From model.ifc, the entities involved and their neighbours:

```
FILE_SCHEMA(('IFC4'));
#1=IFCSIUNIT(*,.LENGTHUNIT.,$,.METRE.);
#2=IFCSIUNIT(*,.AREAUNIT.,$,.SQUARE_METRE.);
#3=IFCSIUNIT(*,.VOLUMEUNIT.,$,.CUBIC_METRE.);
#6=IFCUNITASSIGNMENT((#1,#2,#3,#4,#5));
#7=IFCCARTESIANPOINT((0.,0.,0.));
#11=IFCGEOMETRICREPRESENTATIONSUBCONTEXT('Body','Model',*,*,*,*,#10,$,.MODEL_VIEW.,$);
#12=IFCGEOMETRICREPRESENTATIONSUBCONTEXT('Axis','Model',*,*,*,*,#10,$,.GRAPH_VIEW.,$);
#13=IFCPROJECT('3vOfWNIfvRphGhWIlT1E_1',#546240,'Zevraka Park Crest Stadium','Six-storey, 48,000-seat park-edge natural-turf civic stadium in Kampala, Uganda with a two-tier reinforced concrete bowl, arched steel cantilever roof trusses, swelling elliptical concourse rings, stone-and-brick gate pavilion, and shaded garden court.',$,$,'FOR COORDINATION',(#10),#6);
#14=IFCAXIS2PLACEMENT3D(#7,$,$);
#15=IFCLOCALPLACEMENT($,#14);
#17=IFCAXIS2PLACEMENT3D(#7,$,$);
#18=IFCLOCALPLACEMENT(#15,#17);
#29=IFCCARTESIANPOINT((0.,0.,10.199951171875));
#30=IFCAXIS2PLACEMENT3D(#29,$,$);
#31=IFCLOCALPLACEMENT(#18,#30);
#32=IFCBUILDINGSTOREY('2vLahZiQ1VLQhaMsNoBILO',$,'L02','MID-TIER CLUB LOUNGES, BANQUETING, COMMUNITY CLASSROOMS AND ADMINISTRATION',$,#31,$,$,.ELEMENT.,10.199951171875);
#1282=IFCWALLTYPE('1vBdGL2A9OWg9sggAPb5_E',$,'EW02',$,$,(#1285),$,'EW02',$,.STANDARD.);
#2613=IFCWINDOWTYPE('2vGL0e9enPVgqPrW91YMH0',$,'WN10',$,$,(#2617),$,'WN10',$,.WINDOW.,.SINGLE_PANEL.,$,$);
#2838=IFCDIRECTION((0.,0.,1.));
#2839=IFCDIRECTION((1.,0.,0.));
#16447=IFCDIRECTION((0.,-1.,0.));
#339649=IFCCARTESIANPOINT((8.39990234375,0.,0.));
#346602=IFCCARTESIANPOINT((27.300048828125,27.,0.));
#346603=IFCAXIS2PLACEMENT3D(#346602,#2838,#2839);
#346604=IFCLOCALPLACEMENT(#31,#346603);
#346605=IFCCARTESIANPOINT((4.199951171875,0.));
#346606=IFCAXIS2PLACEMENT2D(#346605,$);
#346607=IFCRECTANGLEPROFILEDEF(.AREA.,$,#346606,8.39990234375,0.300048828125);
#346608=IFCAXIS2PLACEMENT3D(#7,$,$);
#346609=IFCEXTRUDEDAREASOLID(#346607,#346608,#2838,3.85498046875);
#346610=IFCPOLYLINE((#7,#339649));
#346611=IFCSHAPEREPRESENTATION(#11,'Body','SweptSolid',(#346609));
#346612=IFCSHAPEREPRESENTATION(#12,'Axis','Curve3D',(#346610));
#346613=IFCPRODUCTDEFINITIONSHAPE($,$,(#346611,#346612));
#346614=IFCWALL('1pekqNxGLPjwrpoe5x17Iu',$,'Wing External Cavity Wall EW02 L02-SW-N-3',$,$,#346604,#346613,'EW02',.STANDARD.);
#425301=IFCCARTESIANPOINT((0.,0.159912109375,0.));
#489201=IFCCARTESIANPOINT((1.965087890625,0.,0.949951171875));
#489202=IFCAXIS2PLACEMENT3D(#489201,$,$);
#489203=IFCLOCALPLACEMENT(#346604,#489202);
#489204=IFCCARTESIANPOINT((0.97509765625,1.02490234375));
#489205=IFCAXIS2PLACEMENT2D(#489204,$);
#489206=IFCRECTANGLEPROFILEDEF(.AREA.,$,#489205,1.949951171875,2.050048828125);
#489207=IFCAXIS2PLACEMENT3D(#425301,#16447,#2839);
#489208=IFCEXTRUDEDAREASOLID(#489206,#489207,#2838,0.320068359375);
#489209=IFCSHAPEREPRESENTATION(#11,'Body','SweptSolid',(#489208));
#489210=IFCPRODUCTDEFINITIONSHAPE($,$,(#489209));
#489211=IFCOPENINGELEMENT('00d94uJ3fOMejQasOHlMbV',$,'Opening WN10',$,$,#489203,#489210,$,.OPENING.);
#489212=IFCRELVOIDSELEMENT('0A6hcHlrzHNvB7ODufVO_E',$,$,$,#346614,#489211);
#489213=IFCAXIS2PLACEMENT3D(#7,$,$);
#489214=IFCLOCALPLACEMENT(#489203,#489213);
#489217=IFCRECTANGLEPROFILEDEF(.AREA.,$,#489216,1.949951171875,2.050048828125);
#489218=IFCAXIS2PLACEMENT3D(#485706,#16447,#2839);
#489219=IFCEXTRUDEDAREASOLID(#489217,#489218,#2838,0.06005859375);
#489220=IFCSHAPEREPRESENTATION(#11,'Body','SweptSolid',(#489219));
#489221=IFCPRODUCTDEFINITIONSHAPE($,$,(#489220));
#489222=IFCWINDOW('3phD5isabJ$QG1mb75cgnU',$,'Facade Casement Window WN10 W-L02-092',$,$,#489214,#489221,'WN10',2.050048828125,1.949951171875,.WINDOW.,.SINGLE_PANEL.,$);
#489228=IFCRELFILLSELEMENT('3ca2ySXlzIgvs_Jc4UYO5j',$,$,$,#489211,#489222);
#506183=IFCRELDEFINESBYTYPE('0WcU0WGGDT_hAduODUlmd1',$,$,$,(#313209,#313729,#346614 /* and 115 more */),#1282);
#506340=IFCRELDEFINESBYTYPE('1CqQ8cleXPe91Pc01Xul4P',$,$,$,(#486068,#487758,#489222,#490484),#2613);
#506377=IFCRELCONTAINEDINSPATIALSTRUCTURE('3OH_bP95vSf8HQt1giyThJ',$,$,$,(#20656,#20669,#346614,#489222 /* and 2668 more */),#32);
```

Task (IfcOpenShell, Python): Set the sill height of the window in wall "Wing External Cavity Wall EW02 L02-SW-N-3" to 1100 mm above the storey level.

```python
import numpy as np
import ifcopenshell
import ifcopenshell.api.geometry
import ifcopenshell.geom
import ifcopenshell.util.element
import ifcopenshell.util.placement
import ifcopenshell.util.shape
import ifcopenshell.util.unit

model = ifcopenshell.open("model.ifc")
unit_scale = ifcopenshell.util.unit.calculate_unit_scale(model)

window = model.by_guid("3phD5isabJ$QG1mb75cgnU")
opening = window.FillsVoids[0].RelatingOpeningElement
storey = ifcopenshell.util.element.get_container(window, ifc_class="IfcBuildingStorey")
level = ifcopenshell.util.placement.get_local_placement(storey.ObjectPlacement)[2, 3]

# The opening's origin need not be at the sill, so measure its lowest point.
shape = ifcopenshell.geom.create_shape(ifcopenshell.geom.settings(), opening)
bottom = ifcopenshell.util.shape.get_shape_bottom_elevation(shape, shape.geometry) / unit_scale
dz = level + 1.1 - bottom

shift = np.array([0.0, 0.0, dz])
# The window is placed relative to its opening, so it follows when the opening moves.
matrix = ifcopenshell.util.placement.get_local_placement(opening.ObjectPlacement)
matrix[:3, 3] += shift
ifcopenshell.api.geometry.edit_object_placement(
    model, product=opening, matrix=matrix, is_si=False, should_transform_children=True
)

print(f"moved by {dz * unit_scale:+.3f} m")

model.write("model_v2.ifc")
```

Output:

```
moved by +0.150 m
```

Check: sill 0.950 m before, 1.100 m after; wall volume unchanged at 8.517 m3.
